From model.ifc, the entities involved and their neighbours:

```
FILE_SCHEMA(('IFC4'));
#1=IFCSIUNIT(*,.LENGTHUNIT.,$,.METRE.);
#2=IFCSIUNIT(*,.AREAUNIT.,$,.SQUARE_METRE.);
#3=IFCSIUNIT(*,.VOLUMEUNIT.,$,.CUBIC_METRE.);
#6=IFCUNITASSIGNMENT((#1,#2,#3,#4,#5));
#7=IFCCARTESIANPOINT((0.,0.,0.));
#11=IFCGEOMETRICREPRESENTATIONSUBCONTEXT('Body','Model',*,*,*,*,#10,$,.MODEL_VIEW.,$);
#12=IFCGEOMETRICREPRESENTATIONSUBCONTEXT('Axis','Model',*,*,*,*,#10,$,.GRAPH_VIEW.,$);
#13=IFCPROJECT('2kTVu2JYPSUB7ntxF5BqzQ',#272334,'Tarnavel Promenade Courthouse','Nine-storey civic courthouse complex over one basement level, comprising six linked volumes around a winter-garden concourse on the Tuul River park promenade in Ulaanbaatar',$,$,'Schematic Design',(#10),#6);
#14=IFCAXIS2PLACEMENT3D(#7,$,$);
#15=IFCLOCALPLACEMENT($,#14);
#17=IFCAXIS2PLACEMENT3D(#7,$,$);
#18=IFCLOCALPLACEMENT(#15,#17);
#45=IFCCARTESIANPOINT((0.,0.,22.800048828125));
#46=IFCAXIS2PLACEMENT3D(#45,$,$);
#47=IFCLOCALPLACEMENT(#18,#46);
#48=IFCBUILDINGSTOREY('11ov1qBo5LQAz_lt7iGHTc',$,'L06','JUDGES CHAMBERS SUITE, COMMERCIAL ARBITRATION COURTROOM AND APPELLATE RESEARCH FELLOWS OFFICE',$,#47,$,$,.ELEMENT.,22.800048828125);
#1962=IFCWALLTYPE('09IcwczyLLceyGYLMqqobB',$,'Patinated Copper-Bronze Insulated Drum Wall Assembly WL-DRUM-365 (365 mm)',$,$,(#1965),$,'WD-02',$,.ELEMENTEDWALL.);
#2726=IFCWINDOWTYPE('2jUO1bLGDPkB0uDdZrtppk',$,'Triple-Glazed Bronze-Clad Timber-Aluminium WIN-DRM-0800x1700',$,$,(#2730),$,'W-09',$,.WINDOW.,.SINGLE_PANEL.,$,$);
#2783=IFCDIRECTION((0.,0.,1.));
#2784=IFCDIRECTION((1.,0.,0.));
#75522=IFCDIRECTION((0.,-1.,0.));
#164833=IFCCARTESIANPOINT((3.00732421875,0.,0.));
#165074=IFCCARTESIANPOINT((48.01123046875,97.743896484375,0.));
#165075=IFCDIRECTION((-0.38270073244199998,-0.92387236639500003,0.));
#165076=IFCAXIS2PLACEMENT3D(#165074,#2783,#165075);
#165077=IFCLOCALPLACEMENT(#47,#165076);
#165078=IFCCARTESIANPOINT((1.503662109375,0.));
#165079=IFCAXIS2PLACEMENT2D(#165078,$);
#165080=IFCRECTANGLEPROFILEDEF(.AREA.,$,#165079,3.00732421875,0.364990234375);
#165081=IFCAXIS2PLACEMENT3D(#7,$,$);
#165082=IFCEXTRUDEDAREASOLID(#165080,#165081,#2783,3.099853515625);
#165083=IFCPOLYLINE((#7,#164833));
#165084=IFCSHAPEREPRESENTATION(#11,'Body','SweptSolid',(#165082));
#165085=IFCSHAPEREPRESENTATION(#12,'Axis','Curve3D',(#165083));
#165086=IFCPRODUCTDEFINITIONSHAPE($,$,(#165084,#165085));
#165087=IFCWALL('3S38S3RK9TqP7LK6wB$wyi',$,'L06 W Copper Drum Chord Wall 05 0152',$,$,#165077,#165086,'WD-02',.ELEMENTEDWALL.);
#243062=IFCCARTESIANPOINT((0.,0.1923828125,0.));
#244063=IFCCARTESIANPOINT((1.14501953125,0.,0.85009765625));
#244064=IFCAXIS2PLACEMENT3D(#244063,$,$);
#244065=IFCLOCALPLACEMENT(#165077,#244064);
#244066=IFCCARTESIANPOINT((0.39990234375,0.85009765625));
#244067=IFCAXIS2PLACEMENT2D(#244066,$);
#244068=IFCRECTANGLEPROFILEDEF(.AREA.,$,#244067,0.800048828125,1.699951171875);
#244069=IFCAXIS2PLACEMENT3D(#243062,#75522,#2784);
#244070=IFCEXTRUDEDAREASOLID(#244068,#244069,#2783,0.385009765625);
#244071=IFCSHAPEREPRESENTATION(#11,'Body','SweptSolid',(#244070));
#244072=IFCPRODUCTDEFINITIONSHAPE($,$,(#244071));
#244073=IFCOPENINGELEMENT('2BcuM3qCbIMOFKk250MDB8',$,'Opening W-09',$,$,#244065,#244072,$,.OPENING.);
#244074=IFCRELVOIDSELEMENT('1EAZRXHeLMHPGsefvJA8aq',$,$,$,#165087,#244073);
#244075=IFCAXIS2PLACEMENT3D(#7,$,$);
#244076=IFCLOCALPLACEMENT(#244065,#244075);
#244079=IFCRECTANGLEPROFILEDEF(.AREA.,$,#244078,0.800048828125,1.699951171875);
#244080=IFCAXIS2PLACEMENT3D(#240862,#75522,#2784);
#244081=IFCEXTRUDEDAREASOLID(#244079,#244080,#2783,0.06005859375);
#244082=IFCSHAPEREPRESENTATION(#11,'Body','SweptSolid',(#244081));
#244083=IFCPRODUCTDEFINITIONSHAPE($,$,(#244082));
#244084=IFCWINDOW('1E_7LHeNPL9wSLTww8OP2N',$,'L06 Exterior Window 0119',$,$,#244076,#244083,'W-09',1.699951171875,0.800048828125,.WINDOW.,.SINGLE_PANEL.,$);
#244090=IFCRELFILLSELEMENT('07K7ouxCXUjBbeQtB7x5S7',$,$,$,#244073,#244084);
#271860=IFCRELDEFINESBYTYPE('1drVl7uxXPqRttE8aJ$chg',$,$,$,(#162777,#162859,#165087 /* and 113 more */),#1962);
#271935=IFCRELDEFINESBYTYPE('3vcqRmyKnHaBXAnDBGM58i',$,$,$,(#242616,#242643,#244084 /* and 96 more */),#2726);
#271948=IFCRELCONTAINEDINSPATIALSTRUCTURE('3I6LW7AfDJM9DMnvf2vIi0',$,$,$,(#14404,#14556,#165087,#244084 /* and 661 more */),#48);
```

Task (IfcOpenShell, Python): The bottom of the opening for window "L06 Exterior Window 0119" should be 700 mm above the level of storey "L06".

```python
import numpy as np
import ifcopenshell
import ifcopenshell.api.geometry
import ifcopenshell.geom
import ifcopenshell.util.element
import ifcopenshell.util.placement
import ifcopenshell.util.shape
import ifcopenshell.util.unit

model = ifcopenshell.open("model.ifc")
unit_scale = ifcopenshell.util.unit.calculate_unit_scale(model)

window = model.by_guid("1E_7LHeNPL9wSLTww8OP2N")
opening = window.FillsVoids[0].RelatingOpeningElement
storey = ifcopenshell.util.element.get_container(window, ifc_class="IfcBuildingStorey")
level = ifcopenshell.util.placement.get_local_placement(storey.ObjectPlacement)[2, 3]

# The opening's origin need not be at the sill, so measure its lowest point.
shape = ifcopenshell.geom.create_shape(ifcopenshell.geom.settings(), opening)
bottom = ifcopenshell.util.shape.get_shape_bottom_elevation(shape, shape.geometry) / unit_scale
dz = level + 0.7 / unit_scale - bottom

shift = np.array([0.0, 0.0, dz])
# The window is placed relative to its opening, so it follows when the opening moves.
matrix = ifcopenshell.util.placement.get_local_placement(opening.ObjectPlacement)
matrix[:3, 3] += shift
ifcopenshell.api.geometry.edit_object_placement(
    model, product=opening, matrix=matrix, is_si=False, should_transform_children=True
)

print(f"moved by {dz * unit_scale:+.3f} m")

model.write("model_rev.ifc")
```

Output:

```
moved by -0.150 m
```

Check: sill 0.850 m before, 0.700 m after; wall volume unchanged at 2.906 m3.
